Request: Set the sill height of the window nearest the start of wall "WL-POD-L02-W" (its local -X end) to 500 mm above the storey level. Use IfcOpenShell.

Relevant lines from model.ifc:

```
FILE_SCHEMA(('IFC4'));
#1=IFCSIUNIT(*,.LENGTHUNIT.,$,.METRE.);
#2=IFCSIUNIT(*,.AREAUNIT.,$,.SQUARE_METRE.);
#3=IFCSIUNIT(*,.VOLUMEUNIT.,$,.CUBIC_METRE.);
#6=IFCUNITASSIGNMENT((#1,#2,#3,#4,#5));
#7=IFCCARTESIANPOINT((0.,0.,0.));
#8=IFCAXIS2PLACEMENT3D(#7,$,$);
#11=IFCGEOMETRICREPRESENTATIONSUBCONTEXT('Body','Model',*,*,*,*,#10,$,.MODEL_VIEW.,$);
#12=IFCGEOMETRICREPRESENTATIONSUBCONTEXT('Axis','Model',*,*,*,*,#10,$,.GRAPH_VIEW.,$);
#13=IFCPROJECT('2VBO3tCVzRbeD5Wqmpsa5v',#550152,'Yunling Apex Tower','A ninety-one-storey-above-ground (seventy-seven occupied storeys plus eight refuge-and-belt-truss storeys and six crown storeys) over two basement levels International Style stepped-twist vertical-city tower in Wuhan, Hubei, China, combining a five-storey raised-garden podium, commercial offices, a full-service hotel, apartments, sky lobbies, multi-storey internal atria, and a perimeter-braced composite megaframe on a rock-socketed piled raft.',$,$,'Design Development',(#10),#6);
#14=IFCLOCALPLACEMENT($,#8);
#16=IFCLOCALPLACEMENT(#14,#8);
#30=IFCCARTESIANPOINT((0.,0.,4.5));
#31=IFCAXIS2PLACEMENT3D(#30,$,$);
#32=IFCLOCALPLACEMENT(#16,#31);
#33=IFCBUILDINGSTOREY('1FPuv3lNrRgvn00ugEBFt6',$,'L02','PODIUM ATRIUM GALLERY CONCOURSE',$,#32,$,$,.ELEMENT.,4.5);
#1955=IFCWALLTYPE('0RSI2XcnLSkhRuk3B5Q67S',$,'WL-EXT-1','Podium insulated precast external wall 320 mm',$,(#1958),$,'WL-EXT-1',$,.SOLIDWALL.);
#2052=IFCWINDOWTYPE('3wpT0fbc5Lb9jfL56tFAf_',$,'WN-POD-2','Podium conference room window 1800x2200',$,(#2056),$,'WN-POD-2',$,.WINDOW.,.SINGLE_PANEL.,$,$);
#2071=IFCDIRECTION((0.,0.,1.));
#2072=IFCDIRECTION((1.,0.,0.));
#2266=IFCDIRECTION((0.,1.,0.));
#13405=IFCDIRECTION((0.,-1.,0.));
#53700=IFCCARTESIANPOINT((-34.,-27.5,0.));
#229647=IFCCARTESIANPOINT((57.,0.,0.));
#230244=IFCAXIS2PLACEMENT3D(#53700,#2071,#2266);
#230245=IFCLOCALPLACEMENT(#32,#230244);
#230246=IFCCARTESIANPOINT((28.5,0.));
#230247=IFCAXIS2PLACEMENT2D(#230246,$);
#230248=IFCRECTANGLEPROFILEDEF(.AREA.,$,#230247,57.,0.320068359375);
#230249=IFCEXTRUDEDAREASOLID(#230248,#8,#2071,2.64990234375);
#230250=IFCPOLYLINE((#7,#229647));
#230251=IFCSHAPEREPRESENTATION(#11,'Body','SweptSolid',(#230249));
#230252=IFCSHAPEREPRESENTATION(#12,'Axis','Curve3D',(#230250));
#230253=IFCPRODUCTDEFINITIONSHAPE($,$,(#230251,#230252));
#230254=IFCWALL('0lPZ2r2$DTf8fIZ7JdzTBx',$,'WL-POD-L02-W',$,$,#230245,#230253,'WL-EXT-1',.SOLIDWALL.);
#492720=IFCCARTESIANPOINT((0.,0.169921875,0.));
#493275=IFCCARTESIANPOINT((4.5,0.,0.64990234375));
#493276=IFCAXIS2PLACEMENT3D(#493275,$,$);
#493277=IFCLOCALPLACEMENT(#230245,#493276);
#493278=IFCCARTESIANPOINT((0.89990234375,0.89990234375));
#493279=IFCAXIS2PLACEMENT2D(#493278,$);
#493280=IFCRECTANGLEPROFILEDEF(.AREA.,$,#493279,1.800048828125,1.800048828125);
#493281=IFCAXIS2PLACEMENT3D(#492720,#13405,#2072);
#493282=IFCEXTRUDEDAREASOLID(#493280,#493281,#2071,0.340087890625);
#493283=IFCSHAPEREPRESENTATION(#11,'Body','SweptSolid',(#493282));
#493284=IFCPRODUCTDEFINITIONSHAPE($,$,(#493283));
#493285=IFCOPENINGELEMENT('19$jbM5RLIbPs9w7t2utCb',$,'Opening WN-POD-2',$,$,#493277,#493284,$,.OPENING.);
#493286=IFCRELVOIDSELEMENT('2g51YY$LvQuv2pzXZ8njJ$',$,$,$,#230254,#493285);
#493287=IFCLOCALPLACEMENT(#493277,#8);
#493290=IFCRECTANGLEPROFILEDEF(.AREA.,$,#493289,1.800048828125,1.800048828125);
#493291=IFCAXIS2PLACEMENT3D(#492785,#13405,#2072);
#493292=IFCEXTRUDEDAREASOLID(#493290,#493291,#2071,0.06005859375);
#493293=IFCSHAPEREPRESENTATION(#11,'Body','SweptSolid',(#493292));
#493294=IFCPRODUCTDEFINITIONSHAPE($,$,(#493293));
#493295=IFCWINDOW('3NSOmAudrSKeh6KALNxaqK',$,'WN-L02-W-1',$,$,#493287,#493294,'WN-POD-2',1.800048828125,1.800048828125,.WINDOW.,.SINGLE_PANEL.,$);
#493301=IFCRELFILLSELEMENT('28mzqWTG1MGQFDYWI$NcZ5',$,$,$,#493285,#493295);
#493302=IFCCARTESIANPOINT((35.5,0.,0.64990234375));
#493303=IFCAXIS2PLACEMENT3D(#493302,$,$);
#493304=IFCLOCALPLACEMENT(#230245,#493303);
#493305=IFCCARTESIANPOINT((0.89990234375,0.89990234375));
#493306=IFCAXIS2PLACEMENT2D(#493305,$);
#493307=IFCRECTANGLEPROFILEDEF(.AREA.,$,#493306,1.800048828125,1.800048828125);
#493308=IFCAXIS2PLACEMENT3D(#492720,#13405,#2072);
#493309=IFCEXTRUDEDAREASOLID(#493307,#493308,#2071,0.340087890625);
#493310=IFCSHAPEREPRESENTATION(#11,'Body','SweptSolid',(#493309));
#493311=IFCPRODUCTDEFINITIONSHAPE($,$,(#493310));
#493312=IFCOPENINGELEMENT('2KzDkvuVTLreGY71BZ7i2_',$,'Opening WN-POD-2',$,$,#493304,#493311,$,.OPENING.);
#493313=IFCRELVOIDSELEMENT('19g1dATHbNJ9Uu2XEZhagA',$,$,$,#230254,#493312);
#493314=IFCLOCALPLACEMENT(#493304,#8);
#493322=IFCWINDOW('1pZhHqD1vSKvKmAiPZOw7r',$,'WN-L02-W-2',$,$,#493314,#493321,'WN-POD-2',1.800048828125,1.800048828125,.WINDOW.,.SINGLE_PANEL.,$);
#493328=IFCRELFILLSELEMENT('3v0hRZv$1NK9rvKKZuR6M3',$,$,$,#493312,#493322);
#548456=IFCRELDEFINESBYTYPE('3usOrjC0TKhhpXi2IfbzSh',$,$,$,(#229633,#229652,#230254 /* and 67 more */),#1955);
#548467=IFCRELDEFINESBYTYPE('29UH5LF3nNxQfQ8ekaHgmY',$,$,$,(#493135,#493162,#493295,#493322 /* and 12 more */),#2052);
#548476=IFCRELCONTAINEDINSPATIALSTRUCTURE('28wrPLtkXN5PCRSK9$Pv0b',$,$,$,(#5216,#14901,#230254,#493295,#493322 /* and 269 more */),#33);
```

```python
import numpy as np
import ifcopenshell
import ifcopenshell.api.geometry
import ifcopenshell.geom
import ifcopenshell.util.element
import ifcopenshell.util.placement
import ifcopenshell.util.shape
import ifcopenshell.util.unit

model = ifcopenshell.open("model.ifc")
unit_scale = ifcopenshell.util.unit.calculate_unit_scale(model)

window = model.by_guid("3NSOmAudrSKeh6KALNxaqK")
opening = window.FillsVoids[0].RelatingOpeningElement
storey = ifcopenshell.util.element.get_container(window, ifc_class="IfcBuildingStorey")
level = ifcopenshell.util.placement.get_local_placement(storey.ObjectPlacement)[2, 3]

# The opening's origin need not be at the sill, so measure its lowest point.
shape = ifcopenshell.geom.create_shape(ifcopenshell.geom.settings(), opening)
bottom = ifcopenshell.util.shape.get_shape_bottom_elevation(shape, shape.geometry) / unit_scale
dz = level + 0.5 / unit_scale - bottom

shift = np.array([0.0, 0.0, dz])
# The window is placed relative to its opening, so it follows when the opening moves.
matrix = ifcopenshell.util.placement.get_local_placement(opening.ObjectPlacement)
matrix[:3, 3] += shift
ifcopenshell.api.geometry.edit_object_placement(
    model, product=opening, matrix=matrix, is_si=False, should_transform_children=True
)

print(f"moved by {dz * unit_scale:+.3f} m")

model.write("model_v2.ifc")
```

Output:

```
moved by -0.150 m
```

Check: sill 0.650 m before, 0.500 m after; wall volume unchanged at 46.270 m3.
